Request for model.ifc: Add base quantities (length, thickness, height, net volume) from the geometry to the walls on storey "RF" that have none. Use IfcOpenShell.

First a look at what the model holds.

```python
import ifcopenshell
import ifcopenshell.util.element
import ifcopenshell.util.unit

model = ifcopenshell.open("model.ifc")
print(model.schema)
for unit_type in ("LENGTHUNIT", "AREAUNIT", "VOLUMEUNIT"):
    print(unit_type, ifcopenshell.util.unit.calculate_unit_scale(model, unit_type))
storey = next(s for s in model.by_type("IfcBuildingStorey") if s.Name == "RF")
walls = [e for e in ifcopenshell.util.element.get_decomposition(storey) if e.is_a("IfcWall")]
for e in sorted(walls, key=lambda e: e.id()):
    print(e.id(), e.is_a(), e.Name, list(ifcopenshell.util.element.get_psets(e, qtos_only=True)), sep=" | ")
```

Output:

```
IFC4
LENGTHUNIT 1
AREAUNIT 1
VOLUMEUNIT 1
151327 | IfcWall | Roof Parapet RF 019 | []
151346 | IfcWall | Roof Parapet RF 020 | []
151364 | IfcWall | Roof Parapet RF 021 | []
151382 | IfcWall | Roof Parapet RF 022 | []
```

```python
import ifcopenshell
import ifcopenshell.api.pset
import ifcopenshell.geom
import ifcopenshell.util.element
import ifcopenshell.util.shape
import ifcopenshell.util.unit

model = ifcopenshell.open("model.ifc")
unit_scale = ifcopenshell.util.unit.calculate_unit_scale(model)
volume_scale = ifcopenshell.util.unit.calculate_unit_scale(model, "VOLUMEUNIT")
settings = ifcopenshell.geom.settings()

storey = next(s for s in model.by_type("IfcBuildingStorey") if s.Name == "RF")
walls = [e for e in ifcopenshell.util.element.get_decomposition(storey) if e.is_a("IfcWall")]

for e in sorted(walls, key=lambda e: e.id()):
    if ifcopenshell.util.element.get_psets(e, qtos_only=True, should_inherit=False):
        continue
    # Geometry comes back in metres, in the element's own axes.
    shape = ifcopenshell.geom.create_shape(settings, e)
    values = {
        "Length": ifcopenshell.util.shape.get_x(shape.geometry) / unit_scale,
        "Width": ifcopenshell.util.shape.get_y(shape.geometry) / unit_scale,
        "Height": ifcopenshell.util.shape.get_z(shape.geometry) / unit_scale,
        "NetVolume": ifcopenshell.util.shape.get_volume(shape.geometry) / volume_scale,
    }
    qto = ifcopenshell.api.pset.add_qto(model, product=e, name="Qto_WallBaseQuantities")
    ifcopenshell.api.pset.edit_qto(model, qto=qto, properties=values)
    print(e.id(), {k: round(v, 3) for k, v in values.items()})

model.write("model_rev.ifc")
```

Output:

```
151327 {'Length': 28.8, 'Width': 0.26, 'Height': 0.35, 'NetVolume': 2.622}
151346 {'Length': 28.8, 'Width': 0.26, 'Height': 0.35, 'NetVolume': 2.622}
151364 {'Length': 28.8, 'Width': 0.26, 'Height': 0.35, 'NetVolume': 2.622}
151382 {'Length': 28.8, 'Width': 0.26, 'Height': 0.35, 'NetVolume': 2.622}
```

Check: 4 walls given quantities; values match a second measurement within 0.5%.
